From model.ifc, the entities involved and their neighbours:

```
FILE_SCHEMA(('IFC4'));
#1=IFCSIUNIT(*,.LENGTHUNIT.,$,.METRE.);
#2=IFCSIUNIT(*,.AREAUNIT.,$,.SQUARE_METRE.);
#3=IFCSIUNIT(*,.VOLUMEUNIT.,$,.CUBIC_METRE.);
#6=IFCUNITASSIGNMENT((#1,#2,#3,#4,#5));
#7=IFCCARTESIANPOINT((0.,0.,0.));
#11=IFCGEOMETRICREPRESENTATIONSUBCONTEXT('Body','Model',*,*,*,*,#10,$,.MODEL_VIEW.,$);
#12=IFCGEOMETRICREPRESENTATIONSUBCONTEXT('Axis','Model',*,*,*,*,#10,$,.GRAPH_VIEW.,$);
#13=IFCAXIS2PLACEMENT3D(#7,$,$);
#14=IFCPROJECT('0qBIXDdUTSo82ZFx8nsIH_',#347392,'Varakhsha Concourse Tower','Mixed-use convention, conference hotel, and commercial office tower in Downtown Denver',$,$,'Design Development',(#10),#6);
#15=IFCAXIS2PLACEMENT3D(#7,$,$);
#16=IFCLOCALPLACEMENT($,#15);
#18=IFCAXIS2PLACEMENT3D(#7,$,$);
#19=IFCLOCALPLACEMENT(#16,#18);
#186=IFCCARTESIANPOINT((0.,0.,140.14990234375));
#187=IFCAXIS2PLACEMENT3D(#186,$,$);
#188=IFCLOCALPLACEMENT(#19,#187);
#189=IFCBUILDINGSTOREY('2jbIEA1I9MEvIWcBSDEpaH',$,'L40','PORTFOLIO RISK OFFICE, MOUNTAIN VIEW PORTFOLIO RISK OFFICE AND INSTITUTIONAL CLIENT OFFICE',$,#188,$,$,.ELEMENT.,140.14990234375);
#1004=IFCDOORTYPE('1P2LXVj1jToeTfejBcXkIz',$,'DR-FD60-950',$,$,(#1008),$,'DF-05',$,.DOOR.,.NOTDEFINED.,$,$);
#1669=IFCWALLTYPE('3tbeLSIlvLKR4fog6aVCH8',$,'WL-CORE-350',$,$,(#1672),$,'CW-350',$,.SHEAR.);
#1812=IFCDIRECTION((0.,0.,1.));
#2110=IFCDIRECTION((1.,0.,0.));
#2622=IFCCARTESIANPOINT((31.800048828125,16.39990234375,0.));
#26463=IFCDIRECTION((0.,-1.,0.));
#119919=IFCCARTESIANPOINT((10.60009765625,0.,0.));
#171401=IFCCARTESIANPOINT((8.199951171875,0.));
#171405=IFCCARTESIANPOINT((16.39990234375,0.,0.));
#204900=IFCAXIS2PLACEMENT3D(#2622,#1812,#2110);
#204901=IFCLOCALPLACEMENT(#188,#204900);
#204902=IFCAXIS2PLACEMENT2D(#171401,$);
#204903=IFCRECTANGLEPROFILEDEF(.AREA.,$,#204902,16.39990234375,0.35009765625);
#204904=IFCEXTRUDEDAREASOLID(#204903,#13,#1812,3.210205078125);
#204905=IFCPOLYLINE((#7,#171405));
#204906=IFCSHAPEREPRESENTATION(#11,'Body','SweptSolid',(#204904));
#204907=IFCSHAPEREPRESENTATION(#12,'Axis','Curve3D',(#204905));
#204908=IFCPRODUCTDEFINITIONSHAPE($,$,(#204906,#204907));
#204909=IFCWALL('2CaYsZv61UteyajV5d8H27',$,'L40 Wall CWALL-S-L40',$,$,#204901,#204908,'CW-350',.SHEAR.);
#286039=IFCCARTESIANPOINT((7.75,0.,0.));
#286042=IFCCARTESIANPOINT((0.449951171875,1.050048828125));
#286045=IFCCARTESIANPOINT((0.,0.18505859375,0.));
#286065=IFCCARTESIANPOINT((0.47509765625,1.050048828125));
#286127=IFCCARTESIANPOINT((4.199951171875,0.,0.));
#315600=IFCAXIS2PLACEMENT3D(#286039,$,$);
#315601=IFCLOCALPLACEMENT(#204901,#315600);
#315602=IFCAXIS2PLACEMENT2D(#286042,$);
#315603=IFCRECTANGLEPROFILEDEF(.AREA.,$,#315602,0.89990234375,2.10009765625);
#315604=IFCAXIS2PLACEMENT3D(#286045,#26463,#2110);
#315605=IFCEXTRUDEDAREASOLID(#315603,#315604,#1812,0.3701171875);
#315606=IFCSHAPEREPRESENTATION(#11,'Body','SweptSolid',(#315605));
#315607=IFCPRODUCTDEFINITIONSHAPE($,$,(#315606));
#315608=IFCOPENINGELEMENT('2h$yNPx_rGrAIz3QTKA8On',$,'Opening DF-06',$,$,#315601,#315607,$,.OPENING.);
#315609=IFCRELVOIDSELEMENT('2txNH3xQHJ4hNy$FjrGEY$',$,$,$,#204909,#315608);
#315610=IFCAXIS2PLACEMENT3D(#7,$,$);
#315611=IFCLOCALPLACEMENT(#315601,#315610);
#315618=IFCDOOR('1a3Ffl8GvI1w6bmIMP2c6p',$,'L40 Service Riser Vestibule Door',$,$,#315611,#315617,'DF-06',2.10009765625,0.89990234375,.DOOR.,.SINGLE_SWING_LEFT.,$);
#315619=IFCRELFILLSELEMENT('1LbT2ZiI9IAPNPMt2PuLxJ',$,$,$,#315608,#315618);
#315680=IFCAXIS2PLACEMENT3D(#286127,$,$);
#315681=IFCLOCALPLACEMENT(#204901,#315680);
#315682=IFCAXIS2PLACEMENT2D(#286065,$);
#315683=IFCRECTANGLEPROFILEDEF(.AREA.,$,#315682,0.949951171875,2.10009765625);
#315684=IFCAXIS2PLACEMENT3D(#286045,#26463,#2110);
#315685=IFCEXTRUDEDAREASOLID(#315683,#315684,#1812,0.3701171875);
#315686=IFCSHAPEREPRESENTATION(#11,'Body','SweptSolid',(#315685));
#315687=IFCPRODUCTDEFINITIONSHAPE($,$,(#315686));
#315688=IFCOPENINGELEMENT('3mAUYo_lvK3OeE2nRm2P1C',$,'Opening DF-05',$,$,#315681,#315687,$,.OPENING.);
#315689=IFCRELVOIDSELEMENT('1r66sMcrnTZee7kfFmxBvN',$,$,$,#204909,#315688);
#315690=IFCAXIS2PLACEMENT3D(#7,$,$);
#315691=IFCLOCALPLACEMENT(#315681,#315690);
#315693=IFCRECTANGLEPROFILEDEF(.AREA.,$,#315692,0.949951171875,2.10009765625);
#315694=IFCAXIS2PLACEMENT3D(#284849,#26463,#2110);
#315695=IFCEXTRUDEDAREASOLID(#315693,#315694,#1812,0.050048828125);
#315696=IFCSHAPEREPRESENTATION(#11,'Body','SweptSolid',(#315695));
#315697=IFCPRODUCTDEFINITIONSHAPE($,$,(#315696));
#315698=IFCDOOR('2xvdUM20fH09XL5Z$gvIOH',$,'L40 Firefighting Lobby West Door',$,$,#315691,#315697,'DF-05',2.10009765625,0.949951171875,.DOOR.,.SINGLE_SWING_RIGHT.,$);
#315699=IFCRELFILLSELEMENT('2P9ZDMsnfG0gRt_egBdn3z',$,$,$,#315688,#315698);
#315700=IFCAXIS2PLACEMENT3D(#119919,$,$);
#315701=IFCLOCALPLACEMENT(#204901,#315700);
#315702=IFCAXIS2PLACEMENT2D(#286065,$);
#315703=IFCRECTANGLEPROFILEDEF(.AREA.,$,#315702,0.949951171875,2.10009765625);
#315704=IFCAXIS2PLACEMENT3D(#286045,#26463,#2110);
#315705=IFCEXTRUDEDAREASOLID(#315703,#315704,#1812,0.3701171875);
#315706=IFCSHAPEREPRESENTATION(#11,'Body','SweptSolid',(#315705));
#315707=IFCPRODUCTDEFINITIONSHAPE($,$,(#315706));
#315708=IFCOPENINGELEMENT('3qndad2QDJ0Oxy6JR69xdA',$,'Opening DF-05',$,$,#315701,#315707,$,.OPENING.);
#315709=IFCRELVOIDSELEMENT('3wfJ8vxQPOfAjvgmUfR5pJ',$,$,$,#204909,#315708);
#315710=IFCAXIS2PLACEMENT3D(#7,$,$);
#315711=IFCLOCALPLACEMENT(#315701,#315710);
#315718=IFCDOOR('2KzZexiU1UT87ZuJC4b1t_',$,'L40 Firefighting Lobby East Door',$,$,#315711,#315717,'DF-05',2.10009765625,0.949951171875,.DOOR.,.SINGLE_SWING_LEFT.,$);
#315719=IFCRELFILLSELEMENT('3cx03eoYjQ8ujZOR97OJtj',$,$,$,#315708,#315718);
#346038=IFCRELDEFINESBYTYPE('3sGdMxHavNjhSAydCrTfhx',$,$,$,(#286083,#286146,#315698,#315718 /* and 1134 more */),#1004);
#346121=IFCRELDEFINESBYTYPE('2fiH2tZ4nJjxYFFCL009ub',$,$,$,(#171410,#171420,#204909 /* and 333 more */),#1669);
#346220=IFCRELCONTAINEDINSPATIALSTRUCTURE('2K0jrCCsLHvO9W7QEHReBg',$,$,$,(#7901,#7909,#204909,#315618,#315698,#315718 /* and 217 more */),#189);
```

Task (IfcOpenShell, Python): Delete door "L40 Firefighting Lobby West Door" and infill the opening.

```python
import ifcopenshell
import ifcopenshell.api.feature
import ifcopenshell.api.root
import ifcopenshell.geom
import ifcopenshell.util.shape

model = ifcopenshell.open("model.ifc")
settings = ifcopenshell.geom.settings()


def volume(element):
    """Net volume in cubic metres, openings subtracted."""
    shape = ifcopenshell.geom.create_shape(settings, element)
    return ifcopenshell.util.shape.get_volume(shape.geometry)


door = model.by_guid("2xvdUM20fH09XL5Z$gvIOH")
opening = door.FillsVoids[0].RelatingOpeningElement
wall = opening.VoidsElements[0].RelatingBuildingElement
before = volume(wall)

ifcopenshell.api.root.remove_product(model, product=door)
ifcopenshell.api.feature.remove_feature(model, feature=opening)

after = volume(wall)

print(f"wall volume {before:.3f} -> {after:.3f} m3")

model.write("model-out.ifc")
```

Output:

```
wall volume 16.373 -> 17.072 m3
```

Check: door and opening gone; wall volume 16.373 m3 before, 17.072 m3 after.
